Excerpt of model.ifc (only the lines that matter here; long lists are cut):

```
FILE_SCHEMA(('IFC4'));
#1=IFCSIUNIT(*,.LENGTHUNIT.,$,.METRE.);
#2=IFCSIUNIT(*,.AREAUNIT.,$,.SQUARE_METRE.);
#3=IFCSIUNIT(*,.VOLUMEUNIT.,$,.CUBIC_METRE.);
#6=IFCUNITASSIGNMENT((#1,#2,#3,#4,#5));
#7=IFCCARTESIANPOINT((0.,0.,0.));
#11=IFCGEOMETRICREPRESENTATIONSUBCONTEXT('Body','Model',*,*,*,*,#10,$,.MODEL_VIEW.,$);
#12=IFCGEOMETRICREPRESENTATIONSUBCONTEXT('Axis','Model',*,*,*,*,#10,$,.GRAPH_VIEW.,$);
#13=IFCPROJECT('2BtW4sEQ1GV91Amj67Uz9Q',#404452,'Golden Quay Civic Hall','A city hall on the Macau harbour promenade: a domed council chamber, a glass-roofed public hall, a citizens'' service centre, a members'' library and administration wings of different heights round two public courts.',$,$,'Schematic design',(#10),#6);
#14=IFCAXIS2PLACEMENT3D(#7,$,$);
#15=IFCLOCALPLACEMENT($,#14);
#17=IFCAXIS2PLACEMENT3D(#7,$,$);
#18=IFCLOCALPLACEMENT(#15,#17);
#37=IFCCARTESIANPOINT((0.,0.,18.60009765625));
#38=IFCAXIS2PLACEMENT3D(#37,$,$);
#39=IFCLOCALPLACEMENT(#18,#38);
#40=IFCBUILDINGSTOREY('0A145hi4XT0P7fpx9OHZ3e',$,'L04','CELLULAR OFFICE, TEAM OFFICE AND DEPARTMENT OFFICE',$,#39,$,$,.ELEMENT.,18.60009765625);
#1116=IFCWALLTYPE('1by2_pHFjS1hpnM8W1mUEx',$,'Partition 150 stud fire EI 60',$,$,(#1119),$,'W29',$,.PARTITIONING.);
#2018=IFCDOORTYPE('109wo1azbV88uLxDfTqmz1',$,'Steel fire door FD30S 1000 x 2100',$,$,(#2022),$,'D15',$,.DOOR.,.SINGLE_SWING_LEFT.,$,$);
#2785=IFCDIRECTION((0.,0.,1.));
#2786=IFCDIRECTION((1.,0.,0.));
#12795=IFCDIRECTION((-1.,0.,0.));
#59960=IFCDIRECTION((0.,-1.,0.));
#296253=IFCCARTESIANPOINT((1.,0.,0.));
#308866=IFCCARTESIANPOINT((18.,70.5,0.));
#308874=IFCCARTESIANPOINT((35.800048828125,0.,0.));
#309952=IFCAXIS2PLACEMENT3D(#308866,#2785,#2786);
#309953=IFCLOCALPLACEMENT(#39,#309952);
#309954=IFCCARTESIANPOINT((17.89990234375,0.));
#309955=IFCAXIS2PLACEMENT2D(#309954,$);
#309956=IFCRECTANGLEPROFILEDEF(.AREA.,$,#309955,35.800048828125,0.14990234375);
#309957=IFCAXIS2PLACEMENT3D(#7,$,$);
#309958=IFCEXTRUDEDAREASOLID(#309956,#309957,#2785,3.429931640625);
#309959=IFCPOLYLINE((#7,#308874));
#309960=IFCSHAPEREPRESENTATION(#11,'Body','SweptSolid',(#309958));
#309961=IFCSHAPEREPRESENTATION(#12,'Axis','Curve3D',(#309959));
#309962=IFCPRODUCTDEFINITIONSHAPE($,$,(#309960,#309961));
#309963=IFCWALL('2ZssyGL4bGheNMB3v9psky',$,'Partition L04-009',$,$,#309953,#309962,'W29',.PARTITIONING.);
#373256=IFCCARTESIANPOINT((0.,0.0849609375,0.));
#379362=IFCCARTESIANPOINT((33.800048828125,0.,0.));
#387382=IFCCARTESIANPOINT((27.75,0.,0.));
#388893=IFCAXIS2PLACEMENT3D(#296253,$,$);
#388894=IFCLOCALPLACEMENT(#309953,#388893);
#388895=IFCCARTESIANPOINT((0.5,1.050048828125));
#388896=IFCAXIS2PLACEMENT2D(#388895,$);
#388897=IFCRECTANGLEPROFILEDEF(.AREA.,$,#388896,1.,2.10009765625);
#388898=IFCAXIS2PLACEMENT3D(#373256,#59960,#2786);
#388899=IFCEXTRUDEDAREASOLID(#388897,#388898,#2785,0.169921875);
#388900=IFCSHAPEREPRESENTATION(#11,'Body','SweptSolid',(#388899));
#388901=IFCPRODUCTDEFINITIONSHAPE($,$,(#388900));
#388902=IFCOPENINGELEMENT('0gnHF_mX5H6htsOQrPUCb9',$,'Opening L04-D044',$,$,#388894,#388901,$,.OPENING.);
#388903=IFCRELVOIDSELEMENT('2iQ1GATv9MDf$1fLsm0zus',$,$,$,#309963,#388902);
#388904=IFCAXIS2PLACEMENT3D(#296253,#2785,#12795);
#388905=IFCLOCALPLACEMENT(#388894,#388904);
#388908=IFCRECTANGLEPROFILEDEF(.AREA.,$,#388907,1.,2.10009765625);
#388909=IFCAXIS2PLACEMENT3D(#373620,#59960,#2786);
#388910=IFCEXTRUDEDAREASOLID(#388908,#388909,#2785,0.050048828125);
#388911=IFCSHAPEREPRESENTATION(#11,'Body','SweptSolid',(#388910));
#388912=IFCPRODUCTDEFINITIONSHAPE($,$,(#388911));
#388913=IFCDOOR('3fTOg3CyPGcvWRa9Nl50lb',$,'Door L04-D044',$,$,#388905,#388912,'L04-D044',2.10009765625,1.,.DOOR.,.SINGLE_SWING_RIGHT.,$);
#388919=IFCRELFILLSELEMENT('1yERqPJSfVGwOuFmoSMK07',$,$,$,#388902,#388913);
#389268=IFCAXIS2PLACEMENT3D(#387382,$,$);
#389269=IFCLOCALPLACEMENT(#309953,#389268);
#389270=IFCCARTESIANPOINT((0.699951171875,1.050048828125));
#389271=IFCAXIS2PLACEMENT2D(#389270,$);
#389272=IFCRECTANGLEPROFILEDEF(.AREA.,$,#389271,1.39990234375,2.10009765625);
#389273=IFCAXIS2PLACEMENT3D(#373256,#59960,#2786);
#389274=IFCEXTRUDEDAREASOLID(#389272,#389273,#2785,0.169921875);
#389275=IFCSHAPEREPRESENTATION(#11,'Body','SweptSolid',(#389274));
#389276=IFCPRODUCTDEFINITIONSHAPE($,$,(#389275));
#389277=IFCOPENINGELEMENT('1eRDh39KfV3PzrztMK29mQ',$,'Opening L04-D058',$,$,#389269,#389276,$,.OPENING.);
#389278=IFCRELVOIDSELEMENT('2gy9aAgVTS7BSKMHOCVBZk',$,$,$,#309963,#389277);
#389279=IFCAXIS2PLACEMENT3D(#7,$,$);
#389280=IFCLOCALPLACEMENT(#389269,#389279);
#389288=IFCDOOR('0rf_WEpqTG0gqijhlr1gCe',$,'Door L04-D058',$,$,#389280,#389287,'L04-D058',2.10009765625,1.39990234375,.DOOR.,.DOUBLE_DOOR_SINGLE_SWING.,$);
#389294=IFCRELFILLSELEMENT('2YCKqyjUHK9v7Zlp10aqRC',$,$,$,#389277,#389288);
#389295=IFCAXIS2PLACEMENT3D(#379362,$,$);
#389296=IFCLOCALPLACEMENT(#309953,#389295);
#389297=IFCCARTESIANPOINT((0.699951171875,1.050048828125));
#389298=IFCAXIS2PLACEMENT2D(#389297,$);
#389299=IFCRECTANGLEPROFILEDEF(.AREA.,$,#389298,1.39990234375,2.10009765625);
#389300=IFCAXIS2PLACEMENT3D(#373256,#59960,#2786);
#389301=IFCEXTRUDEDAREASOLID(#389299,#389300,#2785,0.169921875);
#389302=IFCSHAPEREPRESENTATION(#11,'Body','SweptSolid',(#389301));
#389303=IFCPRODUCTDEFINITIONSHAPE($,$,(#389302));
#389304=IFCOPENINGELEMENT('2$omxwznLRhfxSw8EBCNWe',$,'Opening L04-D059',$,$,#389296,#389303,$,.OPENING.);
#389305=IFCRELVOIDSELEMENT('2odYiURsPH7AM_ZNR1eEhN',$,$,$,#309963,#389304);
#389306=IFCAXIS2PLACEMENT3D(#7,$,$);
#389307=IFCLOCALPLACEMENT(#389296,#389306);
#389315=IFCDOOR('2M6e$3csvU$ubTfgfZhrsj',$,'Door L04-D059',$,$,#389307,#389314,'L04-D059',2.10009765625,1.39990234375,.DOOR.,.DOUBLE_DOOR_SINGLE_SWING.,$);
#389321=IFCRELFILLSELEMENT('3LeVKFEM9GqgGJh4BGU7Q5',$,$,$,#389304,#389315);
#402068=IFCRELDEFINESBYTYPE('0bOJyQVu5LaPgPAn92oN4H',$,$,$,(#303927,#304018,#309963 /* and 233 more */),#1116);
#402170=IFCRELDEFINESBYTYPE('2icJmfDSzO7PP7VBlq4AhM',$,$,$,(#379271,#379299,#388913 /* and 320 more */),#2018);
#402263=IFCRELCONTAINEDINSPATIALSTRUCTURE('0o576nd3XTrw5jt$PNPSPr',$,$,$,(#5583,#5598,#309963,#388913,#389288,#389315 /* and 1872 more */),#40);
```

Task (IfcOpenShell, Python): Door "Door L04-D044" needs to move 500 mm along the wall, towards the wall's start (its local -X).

```python
import ifcopenshell
import ifcopenshell.api.geometry
import ifcopenshell.util.placement
import ifcopenshell.util.unit

model = ifcopenshell.open("model.ifc")
unit_scale = ifcopenshell.util.unit.calculate_unit_scale(model)

door = model.by_guid("3fTOg3CyPGcvWRa9Nl50lb")
opening = door.FillsVoids[0].RelatingOpeningElement
wall = opening.VoidsElements[0].RelatingBuildingElement

wall_matrix = ifcopenshell.util.placement.get_local_placement(wall.ObjectPlacement)
shift = wall_matrix[:3, 0] * -0.5 / unit_scale
before = ifcopenshell.util.placement.get_local_placement(door.ObjectPlacement)[:3, 3].copy()

# The door is placed relative to its opening, so it follows when the opening moves.
matrix = ifcopenshell.util.placement.get_local_placement(opening.ObjectPlacement)
matrix[:3, 3] += shift
ifcopenshell.api.geometry.edit_object_placement(
    model, product=opening, matrix=matrix, is_si=False, should_transform_children=True
)

after = ifcopenshell.util.placement.get_local_placement(door.ObjectPlacement)[:3, 3]
print("door moved by", (after - before).round(3) + 0.0)

model.write("model-out.ifc")
```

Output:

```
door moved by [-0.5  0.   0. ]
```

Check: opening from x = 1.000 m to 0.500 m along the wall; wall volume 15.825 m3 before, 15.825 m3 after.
